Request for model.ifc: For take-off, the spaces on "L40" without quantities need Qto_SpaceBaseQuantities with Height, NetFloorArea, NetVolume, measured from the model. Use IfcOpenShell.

First a look at what the model holds.

```python
import ifcopenshell
import ifcopenshell.util.element
import ifcopenshell.util.unit

model = ifcopenshell.open("model.ifc")
print(model.schema)
for unit_type in ("LENGTHUNIT", "AREAUNIT", "VOLUMEUNIT"):
    print(unit_type, ifcopenshell.util.unit.calculate_unit_scale(model, unit_type))
storey = next(s for s in model.by_type("IfcBuildingStorey") if s.Name == "L40")
spaces = [e for e in ifcopenshell.util.element.get_decomposition(storey) if e.is_a("IfcSpace")]
for e in sorted(spaces, key=lambda e: e.id()):
    print(e.id(), e.is_a(), e.Name, list(ifcopenshell.util.element.get_psets(e, qtos_only=True)), sep=" | ")
```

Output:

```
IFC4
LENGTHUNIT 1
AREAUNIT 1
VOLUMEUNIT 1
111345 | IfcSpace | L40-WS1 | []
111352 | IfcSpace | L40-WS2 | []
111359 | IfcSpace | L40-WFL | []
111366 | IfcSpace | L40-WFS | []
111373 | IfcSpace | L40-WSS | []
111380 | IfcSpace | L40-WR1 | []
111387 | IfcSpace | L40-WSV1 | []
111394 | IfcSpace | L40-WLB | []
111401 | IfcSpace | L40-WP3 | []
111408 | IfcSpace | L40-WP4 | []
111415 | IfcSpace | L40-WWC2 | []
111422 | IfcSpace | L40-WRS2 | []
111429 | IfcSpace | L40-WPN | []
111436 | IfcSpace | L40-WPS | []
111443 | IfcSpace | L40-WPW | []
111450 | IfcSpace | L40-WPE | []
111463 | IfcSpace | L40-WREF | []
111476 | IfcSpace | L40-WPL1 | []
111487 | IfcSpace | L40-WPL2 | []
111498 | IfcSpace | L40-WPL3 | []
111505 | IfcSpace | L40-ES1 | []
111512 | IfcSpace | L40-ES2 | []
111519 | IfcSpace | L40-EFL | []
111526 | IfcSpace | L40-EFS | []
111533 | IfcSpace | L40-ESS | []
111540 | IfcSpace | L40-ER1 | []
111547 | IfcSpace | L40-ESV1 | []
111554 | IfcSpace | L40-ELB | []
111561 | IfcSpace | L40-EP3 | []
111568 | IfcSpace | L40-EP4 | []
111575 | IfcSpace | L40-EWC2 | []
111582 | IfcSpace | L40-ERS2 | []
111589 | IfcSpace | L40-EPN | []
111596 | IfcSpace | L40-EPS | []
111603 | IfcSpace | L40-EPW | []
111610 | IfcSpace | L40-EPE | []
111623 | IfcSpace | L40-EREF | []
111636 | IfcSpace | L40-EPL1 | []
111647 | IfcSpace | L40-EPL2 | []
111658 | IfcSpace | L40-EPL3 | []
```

```python
import ifcopenshell
import ifcopenshell.api.pset
import ifcopenshell.geom
import ifcopenshell.util.element
import ifcopenshell.util.shape
import ifcopenshell.util.unit

model = ifcopenshell.open("model.ifc")
unit_scale = ifcopenshell.util.unit.calculate_unit_scale(model)
area_scale = ifcopenshell.util.unit.calculate_unit_scale(model, "AREAUNIT")
volume_scale = ifcopenshell.util.unit.calculate_unit_scale(model, "VOLUMEUNIT")
settings = ifcopenshell.geom.settings()

storey = next(s for s in model.by_type("IfcBuildingStorey") if s.Name == "L40")
spaces = [e for e in ifcopenshell.util.element.get_decomposition(storey) if e.is_a("IfcSpace")]

for e in sorted(spaces, key=lambda e: e.id()):
    if ifcopenshell.util.element.get_psets(e, qtos_only=True, should_inherit=False):
        continue
    # Geometry comes back in metres, in the element's own axes.
    shape = ifcopenshell.geom.create_shape(settings, e)
    values = {
        "Height": ifcopenshell.util.shape.get_z(shape.geometry) / unit_scale,
        "NetFloorArea": ifcopenshell.util.shape.get_footprint_area(shape.geometry) / area_scale,
        "NetVolume": ifcopenshell.util.shape.get_volume(shape.geometry) / volume_scale,
    }
    qto = ifcopenshell.api.pset.add_qto(model, product=e, name="Qto_SpaceBaseQuantities")
    ifcopenshell.api.pset.edit_qto(model, qto=qto, properties=values)
    print(e.id(), {k: round(v, 3) for k, v in values.items()})

model.write("model_v2.ifc")
```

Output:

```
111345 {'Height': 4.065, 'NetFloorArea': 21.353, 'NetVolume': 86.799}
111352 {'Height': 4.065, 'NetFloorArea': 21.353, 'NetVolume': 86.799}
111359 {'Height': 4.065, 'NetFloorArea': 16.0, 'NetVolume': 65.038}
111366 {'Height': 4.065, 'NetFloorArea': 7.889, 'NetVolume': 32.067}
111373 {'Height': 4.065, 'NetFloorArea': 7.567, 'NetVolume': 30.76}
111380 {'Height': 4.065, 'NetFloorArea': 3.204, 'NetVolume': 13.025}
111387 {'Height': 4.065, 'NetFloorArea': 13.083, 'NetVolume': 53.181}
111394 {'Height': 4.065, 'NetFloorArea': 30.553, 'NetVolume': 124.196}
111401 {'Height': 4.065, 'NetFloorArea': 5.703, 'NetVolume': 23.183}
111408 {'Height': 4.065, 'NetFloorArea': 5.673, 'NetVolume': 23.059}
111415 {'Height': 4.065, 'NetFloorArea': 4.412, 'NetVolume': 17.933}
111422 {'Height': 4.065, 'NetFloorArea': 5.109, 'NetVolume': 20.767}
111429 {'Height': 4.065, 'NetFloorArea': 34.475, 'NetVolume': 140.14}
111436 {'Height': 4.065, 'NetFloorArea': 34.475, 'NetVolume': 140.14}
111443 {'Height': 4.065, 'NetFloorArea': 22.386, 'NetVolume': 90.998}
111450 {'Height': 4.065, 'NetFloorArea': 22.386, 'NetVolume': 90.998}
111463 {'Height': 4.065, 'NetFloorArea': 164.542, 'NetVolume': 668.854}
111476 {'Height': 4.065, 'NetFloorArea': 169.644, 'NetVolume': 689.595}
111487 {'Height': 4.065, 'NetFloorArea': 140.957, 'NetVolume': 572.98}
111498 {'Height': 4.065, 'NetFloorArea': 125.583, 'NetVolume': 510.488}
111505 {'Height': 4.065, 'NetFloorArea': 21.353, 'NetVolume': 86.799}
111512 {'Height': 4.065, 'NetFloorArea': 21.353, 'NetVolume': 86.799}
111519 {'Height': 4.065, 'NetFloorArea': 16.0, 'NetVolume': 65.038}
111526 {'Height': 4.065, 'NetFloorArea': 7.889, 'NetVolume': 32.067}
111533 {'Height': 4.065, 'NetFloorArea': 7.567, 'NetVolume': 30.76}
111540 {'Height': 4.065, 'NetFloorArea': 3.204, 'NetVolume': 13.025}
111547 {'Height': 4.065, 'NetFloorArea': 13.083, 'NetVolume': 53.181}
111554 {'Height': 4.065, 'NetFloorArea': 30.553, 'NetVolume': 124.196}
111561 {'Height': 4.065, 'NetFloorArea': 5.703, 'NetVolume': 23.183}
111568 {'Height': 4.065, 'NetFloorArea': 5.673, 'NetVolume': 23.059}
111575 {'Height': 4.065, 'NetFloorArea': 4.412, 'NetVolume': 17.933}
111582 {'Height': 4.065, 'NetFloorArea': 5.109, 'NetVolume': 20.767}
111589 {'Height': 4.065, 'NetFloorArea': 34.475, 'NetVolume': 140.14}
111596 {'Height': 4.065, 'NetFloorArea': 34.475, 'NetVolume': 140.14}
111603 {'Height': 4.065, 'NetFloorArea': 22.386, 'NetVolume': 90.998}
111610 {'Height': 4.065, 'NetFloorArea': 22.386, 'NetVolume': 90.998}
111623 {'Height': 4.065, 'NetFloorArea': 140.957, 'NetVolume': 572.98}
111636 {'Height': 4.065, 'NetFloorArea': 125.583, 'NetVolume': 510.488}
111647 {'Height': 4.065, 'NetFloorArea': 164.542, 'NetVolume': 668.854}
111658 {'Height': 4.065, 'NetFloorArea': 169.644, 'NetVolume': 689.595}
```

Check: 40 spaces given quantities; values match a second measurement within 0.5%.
